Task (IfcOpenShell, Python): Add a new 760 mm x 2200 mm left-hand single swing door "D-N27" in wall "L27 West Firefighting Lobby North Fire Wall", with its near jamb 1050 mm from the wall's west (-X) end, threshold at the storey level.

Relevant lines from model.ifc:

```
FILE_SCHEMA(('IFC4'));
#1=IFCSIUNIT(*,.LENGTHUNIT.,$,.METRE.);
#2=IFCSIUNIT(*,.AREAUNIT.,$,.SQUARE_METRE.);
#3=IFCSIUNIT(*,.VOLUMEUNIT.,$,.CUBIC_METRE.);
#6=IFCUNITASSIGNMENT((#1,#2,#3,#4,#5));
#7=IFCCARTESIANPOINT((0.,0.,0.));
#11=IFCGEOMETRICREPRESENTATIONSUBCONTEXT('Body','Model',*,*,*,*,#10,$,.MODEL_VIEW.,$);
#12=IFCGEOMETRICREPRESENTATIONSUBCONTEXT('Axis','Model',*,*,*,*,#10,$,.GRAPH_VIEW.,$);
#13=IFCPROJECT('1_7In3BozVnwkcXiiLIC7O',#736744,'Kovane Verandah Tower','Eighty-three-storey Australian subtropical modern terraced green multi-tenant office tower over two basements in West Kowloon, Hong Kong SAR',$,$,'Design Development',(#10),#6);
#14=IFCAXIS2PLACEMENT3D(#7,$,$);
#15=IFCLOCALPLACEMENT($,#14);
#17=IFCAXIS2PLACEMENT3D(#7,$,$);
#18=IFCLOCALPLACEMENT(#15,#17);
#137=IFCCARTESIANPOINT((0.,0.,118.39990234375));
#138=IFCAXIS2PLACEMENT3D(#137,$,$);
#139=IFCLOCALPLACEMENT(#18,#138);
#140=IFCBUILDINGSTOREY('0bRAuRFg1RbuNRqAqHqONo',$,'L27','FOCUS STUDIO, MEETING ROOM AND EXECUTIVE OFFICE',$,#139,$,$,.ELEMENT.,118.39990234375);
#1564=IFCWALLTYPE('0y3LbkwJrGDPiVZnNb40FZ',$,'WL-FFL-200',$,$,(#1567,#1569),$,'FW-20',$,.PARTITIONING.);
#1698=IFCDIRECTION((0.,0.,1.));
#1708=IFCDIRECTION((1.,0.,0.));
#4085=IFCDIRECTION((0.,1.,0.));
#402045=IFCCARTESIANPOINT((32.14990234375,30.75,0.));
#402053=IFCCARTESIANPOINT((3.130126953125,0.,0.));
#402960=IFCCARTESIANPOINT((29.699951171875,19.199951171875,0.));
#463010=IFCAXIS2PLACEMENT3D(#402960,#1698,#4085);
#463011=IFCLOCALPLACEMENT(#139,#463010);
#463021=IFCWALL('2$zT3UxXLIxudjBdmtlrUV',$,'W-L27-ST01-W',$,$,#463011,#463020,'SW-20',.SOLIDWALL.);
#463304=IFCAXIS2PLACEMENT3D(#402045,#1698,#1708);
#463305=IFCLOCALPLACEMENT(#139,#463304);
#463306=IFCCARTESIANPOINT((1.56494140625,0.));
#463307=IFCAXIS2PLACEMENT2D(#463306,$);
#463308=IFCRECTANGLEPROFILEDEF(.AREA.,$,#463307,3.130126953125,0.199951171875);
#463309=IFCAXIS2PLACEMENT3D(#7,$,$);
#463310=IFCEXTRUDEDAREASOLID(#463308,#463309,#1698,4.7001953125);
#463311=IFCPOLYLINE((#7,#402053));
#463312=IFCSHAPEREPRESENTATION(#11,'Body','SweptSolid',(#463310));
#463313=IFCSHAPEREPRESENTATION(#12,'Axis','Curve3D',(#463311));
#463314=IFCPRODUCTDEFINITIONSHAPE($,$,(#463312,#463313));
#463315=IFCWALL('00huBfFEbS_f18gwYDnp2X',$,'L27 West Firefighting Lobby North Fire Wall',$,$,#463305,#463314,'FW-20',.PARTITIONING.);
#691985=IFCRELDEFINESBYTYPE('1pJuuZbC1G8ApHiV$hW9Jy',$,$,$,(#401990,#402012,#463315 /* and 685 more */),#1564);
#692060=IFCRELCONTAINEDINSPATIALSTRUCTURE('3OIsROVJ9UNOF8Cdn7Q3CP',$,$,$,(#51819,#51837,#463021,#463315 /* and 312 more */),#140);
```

```python
import numpy as np
import ifcopenshell
import ifcopenshell.api.feature
import ifcopenshell.api.geometry
import ifcopenshell.api.root
import ifcopenshell.api.spatial
import ifcopenshell.geom
import ifcopenshell.util.element
import ifcopenshell.util.placement
import ifcopenshell.util.representation
import ifcopenshell.util.shape
import ifcopenshell.util.unit

model = ifcopenshell.open("model.ifc")
unit_scale = ifcopenshell.util.unit.calculate_unit_scale(model)
settings = ifcopenshell.geom.settings()


def volume(element):
    """Net volume in cubic metres, openings subtracted."""
    shape = ifcopenshell.geom.create_shape(settings, element)
    return ifcopenshell.util.shape.get_volume(shape.geometry)


wall = model.by_guid("00huBfFEbS_f18gwYDnp2X")
storey = ifcopenshell.util.element.get_container(wall, ifc_class="IfcBuildingStorey")
context = ifcopenshell.util.representation.get_context(model, "Model", "Body", "MODEL_VIEW")
before = volume(wall)

width, height, from_end, sill = 0.76, 2.2, 1.05, 0.0  # metres

# The wall runs along its own X axis, and the end named is its -X end.
wall_shape = ifcopenshell.geom.create_shape(settings, wall)
x, y, z = ifcopenshell.util.shape.get_vertices(wall_shape.geometry).T
start = x.min() + from_end
face, thickness = float(y.min()), float(y.max() - y.min())
wall_matrix = ifcopenshell.util.placement.get_local_placement(wall.ObjectPlacement)
level = ifcopenshell.util.placement.get_local_placement(storey.ObjectPlacement)[2, 3]


def in_wall(x, y):
    """Placement at x, y metres in the wall's axes, at sill height."""
    matrix = wall_matrix.copy()
    matrix[:, 3] = wall_matrix @ np.array([x / unit_scale, y / unit_scale, 0.0, 1.0])
    matrix[2, 3] = level + sill / unit_scale
    return matrix


# Opening: a box that overshoots both wall faces by 50 mm.
opening = ifcopenshell.api.root.create_entity(model, ifc_class="IfcOpeningElement", predefined_type="OPENING")
box = ifcopenshell.api.geometry.add_wall_representation(
    model, context=context, length=width, height=height, thickness=thickness + 0.1
)
ifcopenshell.api.geometry.assign_representation(model, product=opening, representation=box)
ifcopenshell.api.geometry.edit_object_placement(model, product=opening, matrix=in_wall(start, face - 0.05), is_si=False)
ifcopenshell.api.feature.add_feature(model, feature=opening, element=wall)

door = ifcopenshell.api.root.create_entity(model, ifc_class="IfcDoor", name="D-N27", predefined_type="DOOR")
door.OverallWidth, door.OverallHeight = width / unit_scale, height / unit_scale
door.OperationType = "SINGLE_SWING_LEFT"
body = ifcopenshell.api.geometry.add_door_representation(
    model,
    context=context,
    overall_width=door.OverallWidth,
    overall_height=door.OverallHeight,
    operation_type="SINGLE_SWING_LEFT",
    lining_properties={"LiningDepth": thickness / unit_scale, "ThresholdDepth": thickness / unit_scale},
)
ifcopenshell.api.geometry.assign_representation(model, product=door, representation=body)
ifcopenshell.api.spatial.assign_container(model, products=[door], relating_structure=storey)
ifcopenshell.api.feature.add_filling(model, opening=opening, element=door)

# The lining spans the wall, so the door starts at the wall face.
ifcopenshell.api.geometry.edit_object_placement(model, product=door, matrix=in_wall(start, face), is_si=False)

after = volume(wall)

print(f"wall volume {before:.3f} -> {after:.3f} m3")

model.write("model_rev.ifc")
```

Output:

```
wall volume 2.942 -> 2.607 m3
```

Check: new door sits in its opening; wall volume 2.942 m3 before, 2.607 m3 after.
